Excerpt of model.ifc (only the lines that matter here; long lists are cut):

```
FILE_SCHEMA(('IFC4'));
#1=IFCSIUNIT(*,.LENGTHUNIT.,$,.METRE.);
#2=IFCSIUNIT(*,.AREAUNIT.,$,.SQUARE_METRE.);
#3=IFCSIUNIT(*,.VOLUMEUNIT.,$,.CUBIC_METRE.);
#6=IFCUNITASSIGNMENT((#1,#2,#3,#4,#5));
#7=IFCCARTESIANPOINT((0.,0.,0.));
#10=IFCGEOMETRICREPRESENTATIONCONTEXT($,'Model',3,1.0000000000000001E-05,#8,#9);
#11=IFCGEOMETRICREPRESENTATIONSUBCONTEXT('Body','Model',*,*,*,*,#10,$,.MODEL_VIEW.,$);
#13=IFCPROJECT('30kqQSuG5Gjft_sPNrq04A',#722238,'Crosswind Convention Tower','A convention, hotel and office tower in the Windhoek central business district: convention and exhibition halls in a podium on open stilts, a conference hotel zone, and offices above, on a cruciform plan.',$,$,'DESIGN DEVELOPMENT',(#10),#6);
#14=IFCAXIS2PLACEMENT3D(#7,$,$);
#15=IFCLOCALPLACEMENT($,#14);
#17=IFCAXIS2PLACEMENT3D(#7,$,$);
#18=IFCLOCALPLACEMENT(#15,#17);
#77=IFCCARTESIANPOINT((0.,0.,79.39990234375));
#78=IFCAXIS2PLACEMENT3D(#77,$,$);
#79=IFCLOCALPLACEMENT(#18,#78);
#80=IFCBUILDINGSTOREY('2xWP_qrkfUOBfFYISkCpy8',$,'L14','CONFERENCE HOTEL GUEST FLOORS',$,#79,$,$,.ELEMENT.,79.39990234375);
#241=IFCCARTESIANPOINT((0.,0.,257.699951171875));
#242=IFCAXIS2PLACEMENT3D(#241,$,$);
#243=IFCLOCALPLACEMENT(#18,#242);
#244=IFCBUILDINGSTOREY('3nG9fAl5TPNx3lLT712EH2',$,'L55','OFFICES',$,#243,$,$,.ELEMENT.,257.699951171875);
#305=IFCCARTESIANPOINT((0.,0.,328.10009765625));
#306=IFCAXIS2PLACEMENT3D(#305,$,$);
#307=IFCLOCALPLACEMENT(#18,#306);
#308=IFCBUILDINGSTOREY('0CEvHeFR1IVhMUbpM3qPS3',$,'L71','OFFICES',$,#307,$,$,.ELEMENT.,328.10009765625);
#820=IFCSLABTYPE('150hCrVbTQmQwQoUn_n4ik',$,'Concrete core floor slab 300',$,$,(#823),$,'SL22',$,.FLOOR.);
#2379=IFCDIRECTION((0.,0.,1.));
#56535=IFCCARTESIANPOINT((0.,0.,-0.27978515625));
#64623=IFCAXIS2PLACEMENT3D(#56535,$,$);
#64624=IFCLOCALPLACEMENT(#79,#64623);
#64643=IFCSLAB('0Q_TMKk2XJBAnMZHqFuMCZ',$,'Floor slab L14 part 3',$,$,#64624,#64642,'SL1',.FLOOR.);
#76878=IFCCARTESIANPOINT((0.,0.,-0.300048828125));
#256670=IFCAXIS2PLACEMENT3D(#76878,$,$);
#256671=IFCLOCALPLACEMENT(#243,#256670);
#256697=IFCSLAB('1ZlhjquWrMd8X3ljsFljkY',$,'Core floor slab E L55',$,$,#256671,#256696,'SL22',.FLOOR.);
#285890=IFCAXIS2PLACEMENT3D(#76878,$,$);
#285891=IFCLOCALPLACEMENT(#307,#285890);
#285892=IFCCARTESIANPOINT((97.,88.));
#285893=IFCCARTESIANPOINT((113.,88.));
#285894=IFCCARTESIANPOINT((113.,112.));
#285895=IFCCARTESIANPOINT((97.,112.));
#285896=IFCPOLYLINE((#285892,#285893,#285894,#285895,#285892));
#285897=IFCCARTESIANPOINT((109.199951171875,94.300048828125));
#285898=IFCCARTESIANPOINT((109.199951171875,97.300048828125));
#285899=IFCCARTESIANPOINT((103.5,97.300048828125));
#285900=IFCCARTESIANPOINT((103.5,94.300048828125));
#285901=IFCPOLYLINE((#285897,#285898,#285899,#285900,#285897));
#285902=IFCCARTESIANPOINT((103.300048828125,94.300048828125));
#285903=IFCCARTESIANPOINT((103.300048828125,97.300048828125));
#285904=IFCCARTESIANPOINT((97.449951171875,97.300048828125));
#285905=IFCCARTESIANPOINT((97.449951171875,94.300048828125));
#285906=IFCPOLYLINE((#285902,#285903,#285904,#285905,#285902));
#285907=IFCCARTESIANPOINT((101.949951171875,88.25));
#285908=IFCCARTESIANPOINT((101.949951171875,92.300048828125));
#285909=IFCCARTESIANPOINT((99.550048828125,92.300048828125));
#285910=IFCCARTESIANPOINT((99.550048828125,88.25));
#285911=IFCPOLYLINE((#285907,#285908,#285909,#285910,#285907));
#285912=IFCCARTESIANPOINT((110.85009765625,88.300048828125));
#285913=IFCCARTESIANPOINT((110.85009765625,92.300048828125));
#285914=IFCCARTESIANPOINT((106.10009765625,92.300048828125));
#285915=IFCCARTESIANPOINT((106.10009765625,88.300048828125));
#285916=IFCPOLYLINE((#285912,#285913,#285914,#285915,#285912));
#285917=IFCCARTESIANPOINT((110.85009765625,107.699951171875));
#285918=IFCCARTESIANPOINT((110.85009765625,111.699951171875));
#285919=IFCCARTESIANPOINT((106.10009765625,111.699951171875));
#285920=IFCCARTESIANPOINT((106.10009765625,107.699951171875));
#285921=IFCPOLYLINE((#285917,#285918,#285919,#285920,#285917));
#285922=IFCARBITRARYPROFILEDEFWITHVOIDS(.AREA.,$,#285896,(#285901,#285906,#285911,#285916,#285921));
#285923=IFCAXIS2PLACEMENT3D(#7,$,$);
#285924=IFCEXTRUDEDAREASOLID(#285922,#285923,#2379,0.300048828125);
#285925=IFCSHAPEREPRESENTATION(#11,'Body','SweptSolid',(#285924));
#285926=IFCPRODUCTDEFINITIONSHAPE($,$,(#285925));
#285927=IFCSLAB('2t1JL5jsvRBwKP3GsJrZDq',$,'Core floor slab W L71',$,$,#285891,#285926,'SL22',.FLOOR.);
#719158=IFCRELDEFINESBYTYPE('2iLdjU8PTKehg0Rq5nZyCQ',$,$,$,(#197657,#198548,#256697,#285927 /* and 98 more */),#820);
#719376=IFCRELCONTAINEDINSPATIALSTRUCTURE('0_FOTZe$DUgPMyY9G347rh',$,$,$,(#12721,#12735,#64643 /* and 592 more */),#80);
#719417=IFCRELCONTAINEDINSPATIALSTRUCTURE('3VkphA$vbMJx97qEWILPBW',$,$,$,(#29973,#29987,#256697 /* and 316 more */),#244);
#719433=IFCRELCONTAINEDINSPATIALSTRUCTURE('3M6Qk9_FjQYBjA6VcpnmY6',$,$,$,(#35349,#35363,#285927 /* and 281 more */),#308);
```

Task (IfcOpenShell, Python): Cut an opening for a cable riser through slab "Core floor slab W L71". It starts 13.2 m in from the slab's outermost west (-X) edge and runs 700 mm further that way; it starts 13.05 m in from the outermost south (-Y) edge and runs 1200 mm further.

```python
import numpy as np
import ifcopenshell
import ifcopenshell.api.feature
import ifcopenshell.api.geometry
import ifcopenshell.api.root
import ifcopenshell.geom
import ifcopenshell.util.placement
import ifcopenshell.util.representation
import ifcopenshell.util.shape
import ifcopenshell.util.unit

model = ifcopenshell.open("model.ifc")
unit_scale = ifcopenshell.util.unit.calculate_unit_scale(model)
settings = ifcopenshell.geom.settings()


def volume(element):
    """Net volume in cubic metres, openings subtracted."""
    shape = ifcopenshell.geom.create_shape(settings, element)
    return ifcopenshell.util.shape.get_volume(shape.geometry)


slab = model.by_guid("2t1JL5jsvRBwKP3GsJrZDq")
before = volume(slab)

# Extent in the slab's own axes, in metres. The edges named are its -X and -Y sides.
slab_shape = ifcopenshell.geom.create_shape(settings, slab)
vertices = ifcopenshell.util.shape.get_vertices(slab_shape.geometry)
x_min, y_min, bottom = vertices.min(axis=0)
top = vertices[:, 2].max()

opening = ifcopenshell.api.root.create_entity(model, ifc_class="IfcOpeningElement", name="Cable riser opening", predefined_type="OPENING")
context = ifcopenshell.util.representation.get_context(model, "Model", "Body", "MODEL_VIEW")
width, depth = 0.7, 1.2
outline = [(0.0, 0.0), (width, 0.0), (width, depth), (0.0, depth), (0.0, 0.0)]
# Overshoot both faces by 50 mm so the cut is clean.
shape = ifcopenshell.api.geometry.add_slab_representation(
    model, context=context, depth=top - bottom + 0.1, polyline=outline
)
ifcopenshell.api.geometry.assign_representation(model, product=opening, representation=shape)

matrix = ifcopenshell.util.placement.get_local_placement(slab.ObjectPlacement)
matrix[:, 3] = matrix @ np.append(np.array([x_min + 13.2, y_min + 13.05, bottom - 0.05]) / unit_scale, 1.0)
ifcopenshell.api.geometry.edit_object_placement(model, product=opening, matrix=matrix, is_si=False)
ifcopenshell.api.feature.add_feature(model, feature=opening, element=slab)

after = volume(slab)

print(f"slab volume {before:.3f} -> {after:.3f} m3")

model.write("model_edited.ifc")
```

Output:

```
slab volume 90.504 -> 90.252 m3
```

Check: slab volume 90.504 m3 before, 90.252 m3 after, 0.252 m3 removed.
